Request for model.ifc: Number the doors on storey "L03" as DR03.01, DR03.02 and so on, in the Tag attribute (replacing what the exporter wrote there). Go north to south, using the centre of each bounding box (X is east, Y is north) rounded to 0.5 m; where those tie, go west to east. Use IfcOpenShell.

First a look at what the model holds.

```python
import ifcopenshell
import ifcopenshell.util.element
import ifcopenshell.util.placement

model = ifcopenshell.open("model.ifc")
print(model.schema)
storey = next(s for s in model.by_type("IfcBuildingStorey") if s.Name == "L03")
doors = [e for e in ifcopenshell.util.element.get_decomposition(storey) if e.is_a("IfcDoor")]
for e in sorted(doors, key=lambda e: e.id()):
    origin = ifcopenshell.util.placement.get_local_placement(e.ObjectPlacement)[:3, 3]
    print(e.id(), e.Tag, e.Name, origin.round(2) + 0.0, sep=" | ")
```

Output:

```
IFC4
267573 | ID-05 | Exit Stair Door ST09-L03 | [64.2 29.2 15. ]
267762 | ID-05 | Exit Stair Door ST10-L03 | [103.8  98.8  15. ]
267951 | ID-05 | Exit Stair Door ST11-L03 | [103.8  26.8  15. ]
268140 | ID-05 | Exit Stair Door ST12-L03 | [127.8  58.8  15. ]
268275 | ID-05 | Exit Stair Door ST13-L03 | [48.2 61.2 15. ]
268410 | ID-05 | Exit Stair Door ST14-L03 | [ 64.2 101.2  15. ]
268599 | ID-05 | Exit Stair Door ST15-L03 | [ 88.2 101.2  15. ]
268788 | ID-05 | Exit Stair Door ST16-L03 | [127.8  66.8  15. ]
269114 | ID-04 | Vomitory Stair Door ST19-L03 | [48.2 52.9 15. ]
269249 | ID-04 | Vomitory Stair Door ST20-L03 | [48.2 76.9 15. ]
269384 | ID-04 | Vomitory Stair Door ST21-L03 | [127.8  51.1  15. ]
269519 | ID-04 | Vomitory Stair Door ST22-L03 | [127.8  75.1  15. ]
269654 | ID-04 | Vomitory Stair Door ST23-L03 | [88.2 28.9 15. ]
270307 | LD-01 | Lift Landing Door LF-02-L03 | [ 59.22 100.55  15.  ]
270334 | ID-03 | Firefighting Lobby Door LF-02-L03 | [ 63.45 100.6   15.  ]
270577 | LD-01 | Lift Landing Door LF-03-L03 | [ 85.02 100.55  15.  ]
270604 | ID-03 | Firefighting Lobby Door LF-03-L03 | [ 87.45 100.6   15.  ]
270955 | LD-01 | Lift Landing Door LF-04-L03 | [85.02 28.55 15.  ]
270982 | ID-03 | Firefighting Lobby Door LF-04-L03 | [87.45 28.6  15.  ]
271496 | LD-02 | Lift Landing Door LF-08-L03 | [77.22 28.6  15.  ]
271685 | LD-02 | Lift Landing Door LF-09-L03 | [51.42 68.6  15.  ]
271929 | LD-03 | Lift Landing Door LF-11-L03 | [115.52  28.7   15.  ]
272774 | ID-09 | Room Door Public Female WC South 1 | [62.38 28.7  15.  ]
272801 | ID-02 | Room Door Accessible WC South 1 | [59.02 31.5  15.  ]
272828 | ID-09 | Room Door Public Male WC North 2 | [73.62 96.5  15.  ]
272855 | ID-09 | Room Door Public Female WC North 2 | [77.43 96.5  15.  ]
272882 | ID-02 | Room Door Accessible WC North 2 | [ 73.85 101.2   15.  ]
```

```python
import ifcopenshell
import ifcopenshell.geom
import ifcopenshell.util.element
import ifcopenshell.util.shape

model = ifcopenshell.open("model.ifc")
settings = ifcopenshell.geom.settings()
settings.set("use-world-coords", True)


def centre(element):
    shape = ifcopenshell.geom.create_shape(settings, element)
    return ifcopenshell.util.shape.get_bbox_centroid(shape.geometry)


storey = next(s for s in model.by_type("IfcBuildingStorey") if s.Name == "L03")
doors = [e for e in ifcopenshell.util.element.get_decomposition(storey) if e.is_a("IfcDoor")]

# Insertion points can sit at a corner or the storey origin, so sort by the geometry (in metres).
centres = {e: centre(e) for e in doors}
doors.sort(key=lambda e: (-round(centres[e][1] / 0.5), centres[e][0]))

for i, e in enumerate(doors, start=1):
    number = f"DR03.{i:02d}"
    e.Tag = number
    print(e.id(), number)

model.write("model-out.ifc")
```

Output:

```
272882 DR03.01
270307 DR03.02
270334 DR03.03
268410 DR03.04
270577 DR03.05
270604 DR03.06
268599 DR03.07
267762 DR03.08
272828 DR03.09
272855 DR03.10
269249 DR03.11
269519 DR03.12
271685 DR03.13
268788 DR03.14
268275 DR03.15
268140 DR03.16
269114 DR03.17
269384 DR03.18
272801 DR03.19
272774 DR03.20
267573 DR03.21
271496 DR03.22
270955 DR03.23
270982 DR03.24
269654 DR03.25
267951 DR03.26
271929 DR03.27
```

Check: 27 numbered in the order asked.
